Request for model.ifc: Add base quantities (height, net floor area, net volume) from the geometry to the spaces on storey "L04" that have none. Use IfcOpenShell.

First a look at what the model holds.

```python
import ifcopenshell
import ifcopenshell.util.element
import ifcopenshell.util.unit

model = ifcopenshell.open("model.ifc")
print(model.schema)
for unit_type in ("LENGTHUNIT", "AREAUNIT", "VOLUMEUNIT"):
    print(unit_type, ifcopenshell.util.unit.calculate_unit_scale(model, unit_type))
storey = next(s for s in model.by_type("IfcBuildingStorey") if s.Name == "L04")
spaces = [e for e in ifcopenshell.util.element.get_decomposition(storey) if e.is_a("IfcSpace")]
for e in sorted(spaces, key=lambda e: e.id()):
    print(e.id(), e.is_a(), e.Name, list(ifcopenshell.util.element.get_psets(e, qtos_only=True)), sep=" | ")
```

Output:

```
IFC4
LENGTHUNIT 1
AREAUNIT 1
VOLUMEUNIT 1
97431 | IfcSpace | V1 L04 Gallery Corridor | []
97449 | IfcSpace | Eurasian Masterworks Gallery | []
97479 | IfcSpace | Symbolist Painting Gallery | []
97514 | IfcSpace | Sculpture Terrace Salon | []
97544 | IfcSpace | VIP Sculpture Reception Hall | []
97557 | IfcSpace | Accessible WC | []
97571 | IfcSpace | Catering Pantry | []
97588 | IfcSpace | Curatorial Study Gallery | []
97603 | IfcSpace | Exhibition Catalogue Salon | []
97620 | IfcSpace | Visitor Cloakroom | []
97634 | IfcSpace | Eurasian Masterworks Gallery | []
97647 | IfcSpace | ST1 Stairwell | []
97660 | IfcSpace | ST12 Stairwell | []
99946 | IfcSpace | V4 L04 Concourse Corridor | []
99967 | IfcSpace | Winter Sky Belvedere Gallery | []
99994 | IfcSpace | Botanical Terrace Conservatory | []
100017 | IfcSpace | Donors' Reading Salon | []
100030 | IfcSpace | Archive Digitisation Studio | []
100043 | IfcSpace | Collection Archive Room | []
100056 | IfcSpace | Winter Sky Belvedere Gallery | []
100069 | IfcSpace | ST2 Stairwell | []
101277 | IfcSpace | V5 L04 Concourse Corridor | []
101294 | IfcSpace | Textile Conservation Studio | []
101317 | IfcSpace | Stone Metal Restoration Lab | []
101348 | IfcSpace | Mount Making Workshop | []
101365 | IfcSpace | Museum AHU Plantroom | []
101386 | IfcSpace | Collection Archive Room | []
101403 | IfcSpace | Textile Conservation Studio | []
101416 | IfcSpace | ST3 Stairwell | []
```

```python
import ifcopenshell
import ifcopenshell.api.pset
import ifcopenshell.geom
import ifcopenshell.util.element
import ifcopenshell.util.shape
import ifcopenshell.util.unit

model = ifcopenshell.open("model.ifc")
unit_scale = ifcopenshell.util.unit.calculate_unit_scale(model)
area_scale = ifcopenshell.util.unit.calculate_unit_scale(model, "AREAUNIT")
volume_scale = ifcopenshell.util.unit.calculate_unit_scale(model, "VOLUMEUNIT")
settings = ifcopenshell.geom.settings()

storey = next(s for s in model.by_type("IfcBuildingStorey") if s.Name == "L04")
spaces = [e for e in ifcopenshell.util.element.get_decomposition(storey) if e.is_a("IfcSpace")]

for e in sorted(spaces, key=lambda e: e.id()):
    if ifcopenshell.util.element.get_psets(e, qtos_only=True, should_inherit=False):
        continue
    # Geometry comes back in metres, in the element's own axes.
    shape = ifcopenshell.geom.create_shape(settings, e)
    values = {
        "Height": ifcopenshell.util.shape.get_z(shape.geometry) / unit_scale,
        "NetFloorArea": ifcopenshell.util.shape.get_footprint_area(shape.geometry) / area_scale,
        "NetVolume": ifcopenshell.util.shape.get_volume(shape.geometry) / volume_scale,
    }
    qto = ifcopenshell.api.pset.add_qto(model, product=e, name="Qto_SpaceBaseQuantities")
    ifcopenshell.api.pset.edit_qto(model, qto=qto, properties=values)
    print(e.id(), {k: round(v, 3) for k, v in values.items()})

model.write("model_v2.ifc")
```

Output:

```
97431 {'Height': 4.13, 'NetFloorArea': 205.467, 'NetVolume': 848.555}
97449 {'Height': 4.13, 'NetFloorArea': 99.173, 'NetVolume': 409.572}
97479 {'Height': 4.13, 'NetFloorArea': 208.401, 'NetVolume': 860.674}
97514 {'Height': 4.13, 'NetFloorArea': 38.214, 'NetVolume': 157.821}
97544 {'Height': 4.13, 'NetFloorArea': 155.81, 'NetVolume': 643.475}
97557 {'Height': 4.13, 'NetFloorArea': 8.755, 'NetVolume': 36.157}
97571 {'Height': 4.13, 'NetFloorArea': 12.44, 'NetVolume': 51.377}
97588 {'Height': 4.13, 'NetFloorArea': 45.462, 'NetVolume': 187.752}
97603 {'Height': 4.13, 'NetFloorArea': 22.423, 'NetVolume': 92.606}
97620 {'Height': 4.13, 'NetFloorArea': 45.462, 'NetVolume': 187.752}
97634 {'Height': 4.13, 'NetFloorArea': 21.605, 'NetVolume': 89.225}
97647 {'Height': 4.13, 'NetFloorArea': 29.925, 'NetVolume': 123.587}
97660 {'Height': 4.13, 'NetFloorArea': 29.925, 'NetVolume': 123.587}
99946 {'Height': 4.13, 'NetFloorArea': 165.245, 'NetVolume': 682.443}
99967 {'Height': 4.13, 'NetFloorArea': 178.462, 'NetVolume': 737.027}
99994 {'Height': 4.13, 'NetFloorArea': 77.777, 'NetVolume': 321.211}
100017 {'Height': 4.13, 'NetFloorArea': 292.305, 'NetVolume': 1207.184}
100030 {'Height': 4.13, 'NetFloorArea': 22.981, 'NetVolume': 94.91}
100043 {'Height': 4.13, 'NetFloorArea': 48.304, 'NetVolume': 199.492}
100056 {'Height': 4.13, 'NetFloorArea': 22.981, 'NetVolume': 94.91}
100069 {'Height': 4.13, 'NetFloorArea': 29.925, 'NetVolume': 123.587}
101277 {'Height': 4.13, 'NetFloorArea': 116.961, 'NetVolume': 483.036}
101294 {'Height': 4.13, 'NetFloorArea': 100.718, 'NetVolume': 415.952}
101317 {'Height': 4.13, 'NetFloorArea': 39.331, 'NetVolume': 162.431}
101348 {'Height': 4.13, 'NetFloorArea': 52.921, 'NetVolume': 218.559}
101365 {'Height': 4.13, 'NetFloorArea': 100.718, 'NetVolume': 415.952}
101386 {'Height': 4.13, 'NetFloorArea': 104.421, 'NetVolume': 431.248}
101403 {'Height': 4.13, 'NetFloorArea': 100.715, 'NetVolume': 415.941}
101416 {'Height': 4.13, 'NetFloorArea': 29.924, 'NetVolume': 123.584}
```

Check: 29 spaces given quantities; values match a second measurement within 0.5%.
